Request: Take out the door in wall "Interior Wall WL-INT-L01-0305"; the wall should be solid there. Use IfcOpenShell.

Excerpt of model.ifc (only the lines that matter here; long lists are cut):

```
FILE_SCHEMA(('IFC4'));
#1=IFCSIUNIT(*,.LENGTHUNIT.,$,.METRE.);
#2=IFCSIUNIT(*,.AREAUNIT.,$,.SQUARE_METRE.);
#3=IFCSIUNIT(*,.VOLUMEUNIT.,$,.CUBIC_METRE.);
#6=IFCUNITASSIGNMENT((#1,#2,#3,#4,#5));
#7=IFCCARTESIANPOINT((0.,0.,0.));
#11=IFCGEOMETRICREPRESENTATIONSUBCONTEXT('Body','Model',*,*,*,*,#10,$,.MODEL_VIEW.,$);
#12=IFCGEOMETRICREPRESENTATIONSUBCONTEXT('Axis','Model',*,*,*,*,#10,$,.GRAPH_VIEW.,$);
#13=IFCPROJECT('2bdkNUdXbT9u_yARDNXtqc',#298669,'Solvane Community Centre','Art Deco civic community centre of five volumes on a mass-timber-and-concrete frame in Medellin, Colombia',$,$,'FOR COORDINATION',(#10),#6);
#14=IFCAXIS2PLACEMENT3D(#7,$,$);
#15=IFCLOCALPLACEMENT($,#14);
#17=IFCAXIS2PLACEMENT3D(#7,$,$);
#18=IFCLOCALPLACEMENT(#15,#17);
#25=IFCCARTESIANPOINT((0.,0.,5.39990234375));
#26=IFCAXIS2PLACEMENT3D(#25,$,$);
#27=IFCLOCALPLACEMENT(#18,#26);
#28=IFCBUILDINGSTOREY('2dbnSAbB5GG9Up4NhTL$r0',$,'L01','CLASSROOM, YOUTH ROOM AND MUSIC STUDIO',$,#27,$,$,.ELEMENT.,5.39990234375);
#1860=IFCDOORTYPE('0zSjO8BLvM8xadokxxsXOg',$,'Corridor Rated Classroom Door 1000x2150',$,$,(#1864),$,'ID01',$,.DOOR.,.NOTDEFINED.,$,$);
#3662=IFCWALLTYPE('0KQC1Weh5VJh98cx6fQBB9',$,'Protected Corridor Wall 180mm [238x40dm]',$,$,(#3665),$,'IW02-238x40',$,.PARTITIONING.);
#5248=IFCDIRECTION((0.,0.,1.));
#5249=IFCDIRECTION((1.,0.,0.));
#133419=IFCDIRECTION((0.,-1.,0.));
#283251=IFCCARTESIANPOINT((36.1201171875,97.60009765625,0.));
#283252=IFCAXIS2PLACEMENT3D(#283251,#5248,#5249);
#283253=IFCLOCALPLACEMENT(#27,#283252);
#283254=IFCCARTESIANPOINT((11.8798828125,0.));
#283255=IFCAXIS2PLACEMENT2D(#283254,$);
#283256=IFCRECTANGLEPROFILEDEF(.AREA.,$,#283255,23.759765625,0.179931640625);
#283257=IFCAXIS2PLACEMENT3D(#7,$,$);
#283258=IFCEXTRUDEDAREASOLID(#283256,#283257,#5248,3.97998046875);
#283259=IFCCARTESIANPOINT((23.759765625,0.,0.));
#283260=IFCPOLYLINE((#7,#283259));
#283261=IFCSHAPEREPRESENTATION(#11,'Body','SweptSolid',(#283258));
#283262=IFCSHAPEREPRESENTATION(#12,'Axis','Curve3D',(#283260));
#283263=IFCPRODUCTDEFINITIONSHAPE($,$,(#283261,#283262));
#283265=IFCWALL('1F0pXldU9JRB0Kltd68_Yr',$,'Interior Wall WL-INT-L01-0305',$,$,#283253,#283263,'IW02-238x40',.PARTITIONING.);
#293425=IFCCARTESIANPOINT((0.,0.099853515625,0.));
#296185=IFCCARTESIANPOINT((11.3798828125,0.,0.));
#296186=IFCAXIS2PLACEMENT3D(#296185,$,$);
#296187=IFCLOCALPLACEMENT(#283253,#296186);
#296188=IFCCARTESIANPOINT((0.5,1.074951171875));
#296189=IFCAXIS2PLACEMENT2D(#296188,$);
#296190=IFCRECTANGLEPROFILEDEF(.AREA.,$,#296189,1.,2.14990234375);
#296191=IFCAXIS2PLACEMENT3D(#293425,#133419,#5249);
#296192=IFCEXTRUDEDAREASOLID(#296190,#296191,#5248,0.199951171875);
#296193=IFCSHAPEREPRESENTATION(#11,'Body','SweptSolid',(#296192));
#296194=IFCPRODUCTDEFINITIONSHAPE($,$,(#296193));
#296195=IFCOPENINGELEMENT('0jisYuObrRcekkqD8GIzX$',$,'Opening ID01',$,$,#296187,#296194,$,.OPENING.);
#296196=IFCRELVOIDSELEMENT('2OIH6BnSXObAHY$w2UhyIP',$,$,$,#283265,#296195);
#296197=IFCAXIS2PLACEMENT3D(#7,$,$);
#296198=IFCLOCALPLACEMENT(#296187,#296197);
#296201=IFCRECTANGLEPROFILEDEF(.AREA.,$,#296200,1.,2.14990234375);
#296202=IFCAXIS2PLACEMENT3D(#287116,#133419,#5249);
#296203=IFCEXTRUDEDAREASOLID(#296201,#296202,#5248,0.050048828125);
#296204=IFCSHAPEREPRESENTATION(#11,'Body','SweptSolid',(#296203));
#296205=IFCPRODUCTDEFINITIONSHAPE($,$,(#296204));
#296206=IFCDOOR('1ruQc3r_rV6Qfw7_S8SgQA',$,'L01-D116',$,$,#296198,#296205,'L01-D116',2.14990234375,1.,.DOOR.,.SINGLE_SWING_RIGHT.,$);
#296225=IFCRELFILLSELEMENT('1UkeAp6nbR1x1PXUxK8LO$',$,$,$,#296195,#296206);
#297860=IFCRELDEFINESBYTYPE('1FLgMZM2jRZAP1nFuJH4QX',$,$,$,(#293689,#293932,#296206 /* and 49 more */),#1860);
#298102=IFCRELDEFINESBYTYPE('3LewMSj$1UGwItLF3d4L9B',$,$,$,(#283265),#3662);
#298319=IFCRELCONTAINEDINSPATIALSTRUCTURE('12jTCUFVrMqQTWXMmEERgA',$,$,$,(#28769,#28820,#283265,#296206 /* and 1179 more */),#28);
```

```python
import ifcopenshell
import ifcopenshell.api.feature
import ifcopenshell.api.root
import ifcopenshell.geom
import ifcopenshell.util.shape

model = ifcopenshell.open("model.ifc")
settings = ifcopenshell.geom.settings()


def volume(element):
    """Net volume in cubic metres, openings subtracted."""
    shape = ifcopenshell.geom.create_shape(settings, element)
    return ifcopenshell.util.shape.get_volume(shape.geometry)


door = model.by_guid("1ruQc3r_rV6Qfw7_S8SgQA")
opening = door.FillsVoids[0].RelatingOpeningElement
wall = opening.VoidsElements[0].RelatingBuildingElement
before = volume(wall)

ifcopenshell.api.root.remove_product(model, product=door)
ifcopenshell.api.feature.remove_feature(model, feature=opening)

after = volume(wall)

print(f"wall volume {before:.3f} -> {after:.3f} m3")

model.write("model_rev.ifc")
```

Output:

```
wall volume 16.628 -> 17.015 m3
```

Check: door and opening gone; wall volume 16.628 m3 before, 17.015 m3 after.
